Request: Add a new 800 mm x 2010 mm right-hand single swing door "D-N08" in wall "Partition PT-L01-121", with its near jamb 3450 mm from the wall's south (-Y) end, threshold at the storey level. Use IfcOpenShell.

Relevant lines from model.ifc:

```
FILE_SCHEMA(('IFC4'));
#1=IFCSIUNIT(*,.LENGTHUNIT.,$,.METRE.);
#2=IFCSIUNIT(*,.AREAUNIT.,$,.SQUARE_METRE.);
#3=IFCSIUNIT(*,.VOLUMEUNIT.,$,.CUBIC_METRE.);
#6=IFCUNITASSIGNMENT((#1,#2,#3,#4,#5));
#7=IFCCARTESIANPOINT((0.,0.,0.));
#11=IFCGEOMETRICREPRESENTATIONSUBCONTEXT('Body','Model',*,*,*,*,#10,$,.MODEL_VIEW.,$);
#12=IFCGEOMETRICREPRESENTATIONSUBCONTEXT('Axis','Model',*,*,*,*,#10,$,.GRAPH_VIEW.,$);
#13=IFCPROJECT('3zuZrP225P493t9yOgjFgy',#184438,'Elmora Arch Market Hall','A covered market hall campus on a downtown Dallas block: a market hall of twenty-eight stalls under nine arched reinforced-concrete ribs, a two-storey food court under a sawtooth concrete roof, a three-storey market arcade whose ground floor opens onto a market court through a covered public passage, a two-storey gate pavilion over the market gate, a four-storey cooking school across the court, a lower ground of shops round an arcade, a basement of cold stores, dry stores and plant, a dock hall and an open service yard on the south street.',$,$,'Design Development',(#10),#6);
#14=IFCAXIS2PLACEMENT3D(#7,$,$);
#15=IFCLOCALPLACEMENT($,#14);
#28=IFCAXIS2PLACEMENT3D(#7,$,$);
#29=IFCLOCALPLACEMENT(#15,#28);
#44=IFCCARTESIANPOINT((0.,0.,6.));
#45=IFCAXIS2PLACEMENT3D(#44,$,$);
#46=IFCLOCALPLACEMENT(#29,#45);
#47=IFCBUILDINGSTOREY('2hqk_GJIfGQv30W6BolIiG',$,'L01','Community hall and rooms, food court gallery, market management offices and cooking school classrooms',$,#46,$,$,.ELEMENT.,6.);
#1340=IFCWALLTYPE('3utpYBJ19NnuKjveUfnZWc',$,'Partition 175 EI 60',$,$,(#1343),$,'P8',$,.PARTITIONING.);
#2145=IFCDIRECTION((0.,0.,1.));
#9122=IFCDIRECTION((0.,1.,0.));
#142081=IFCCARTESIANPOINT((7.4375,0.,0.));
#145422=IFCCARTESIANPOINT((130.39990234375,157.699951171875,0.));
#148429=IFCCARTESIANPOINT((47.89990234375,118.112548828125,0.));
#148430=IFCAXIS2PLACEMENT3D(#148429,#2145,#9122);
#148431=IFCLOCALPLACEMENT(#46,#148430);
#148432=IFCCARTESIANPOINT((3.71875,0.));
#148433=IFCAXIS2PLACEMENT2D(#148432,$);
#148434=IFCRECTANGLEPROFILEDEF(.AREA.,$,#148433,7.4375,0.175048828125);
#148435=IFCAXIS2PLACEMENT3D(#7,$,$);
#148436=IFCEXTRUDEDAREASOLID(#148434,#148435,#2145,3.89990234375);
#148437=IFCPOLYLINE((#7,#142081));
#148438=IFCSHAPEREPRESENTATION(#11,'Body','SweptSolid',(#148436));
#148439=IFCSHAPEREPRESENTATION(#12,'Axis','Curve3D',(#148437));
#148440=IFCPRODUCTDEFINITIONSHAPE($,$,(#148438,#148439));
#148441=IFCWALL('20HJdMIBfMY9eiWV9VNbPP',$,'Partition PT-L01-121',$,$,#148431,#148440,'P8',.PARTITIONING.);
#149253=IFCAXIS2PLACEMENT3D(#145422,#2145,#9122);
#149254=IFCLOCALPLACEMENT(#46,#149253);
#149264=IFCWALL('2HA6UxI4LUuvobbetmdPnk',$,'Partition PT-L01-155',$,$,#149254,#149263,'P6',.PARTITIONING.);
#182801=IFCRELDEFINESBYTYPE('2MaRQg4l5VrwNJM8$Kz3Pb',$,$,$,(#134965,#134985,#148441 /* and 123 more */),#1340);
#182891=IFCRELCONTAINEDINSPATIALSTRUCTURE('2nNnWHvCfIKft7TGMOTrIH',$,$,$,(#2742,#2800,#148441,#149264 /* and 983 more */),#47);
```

```python
import numpy as np
import ifcopenshell
import ifcopenshell.api.feature
import ifcopenshell.api.geometry
import ifcopenshell.api.root
import ifcopenshell.api.spatial
import ifcopenshell.geom
import ifcopenshell.util.element
import ifcopenshell.util.placement
import ifcopenshell.util.representation
import ifcopenshell.util.shape
import ifcopenshell.util.unit

model = ifcopenshell.open("model.ifc")
unit_scale = ifcopenshell.util.unit.calculate_unit_scale(model)
settings = ifcopenshell.geom.settings()


def volume(element):
    """Net volume in cubic metres, openings subtracted."""
    shape = ifcopenshell.geom.create_shape(settings, element)
    return ifcopenshell.util.shape.get_volume(shape.geometry)


wall = model.by_id(148441)
storey = ifcopenshell.util.element.get_container(wall, ifc_class="IfcBuildingStorey")
context = ifcopenshell.util.representation.get_context(model, "Model", "Body", "MODEL_VIEW")
before = volume(wall)

width, height, from_end, sill = 0.8, 2.01, 3.45, 0.0  # metres

# The wall runs along its own X axis, and the end named is its -X end.
wall_shape = ifcopenshell.geom.create_shape(settings, wall)
x, y, z = ifcopenshell.util.shape.get_vertices(wall_shape.geometry).T
start = x.min() + from_end
face, thickness = float(y.min()), float(y.max() - y.min())
wall_matrix = ifcopenshell.util.placement.get_local_placement(wall.ObjectPlacement)
level = ifcopenshell.util.placement.get_local_placement(storey.ObjectPlacement)[2, 3]


def in_wall(x, y):
    """Placement at x, y metres in the wall's axes, at sill height."""
    matrix = wall_matrix.copy()
    matrix[:, 3] = wall_matrix @ np.array([x / unit_scale, y / unit_scale, 0.0, 1.0])
    matrix[2, 3] = level + sill / unit_scale
    return matrix


# Opening: a box that overshoots both wall faces by 50 mm.
opening = ifcopenshell.api.root.create_entity(model, ifc_class="IfcOpeningElement", predefined_type="OPENING")
box = ifcopenshell.api.geometry.add_wall_representation(
    model, context=context, length=width, height=height, thickness=thickness + 0.1
)
ifcopenshell.api.geometry.assign_representation(model, product=opening, representation=box)
ifcopenshell.api.geometry.edit_object_placement(model, product=opening, matrix=in_wall(start, face - 0.05), is_si=False)
ifcopenshell.api.feature.add_feature(model, feature=opening, element=wall)

door = ifcopenshell.api.root.create_entity(model, ifc_class="IfcDoor", name="D-N08", predefined_type="DOOR")
door.OverallWidth, door.OverallHeight = width / unit_scale, height / unit_scale
door.OperationType = "SINGLE_SWING_RIGHT"
body = ifcopenshell.api.geometry.add_door_representation(
    model,
    context=context,
    overall_width=door.OverallWidth,
    overall_height=door.OverallHeight,
    operation_type="SINGLE_SWING_RIGHT",
    lining_properties={"LiningDepth": thickness / unit_scale, "ThresholdDepth": thickness / unit_scale},
)
ifcopenshell.api.geometry.assign_representation(model, product=door, representation=body)
ifcopenshell.api.spatial.assign_container(model, products=[door], relating_structure=storey)
ifcopenshell.api.feature.add_filling(model, opening=opening, element=door)

# The lining spans the wall, so the door starts at the wall face.
ifcopenshell.api.geometry.edit_object_placement(model, product=door, matrix=in_wall(start, face), is_si=False)

after = volume(wall)

print(f"wall volume {before:.3f} -> {after:.3f} m3")

model.write("model_rev.ifc")
```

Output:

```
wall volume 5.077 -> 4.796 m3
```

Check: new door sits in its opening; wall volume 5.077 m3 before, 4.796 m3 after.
